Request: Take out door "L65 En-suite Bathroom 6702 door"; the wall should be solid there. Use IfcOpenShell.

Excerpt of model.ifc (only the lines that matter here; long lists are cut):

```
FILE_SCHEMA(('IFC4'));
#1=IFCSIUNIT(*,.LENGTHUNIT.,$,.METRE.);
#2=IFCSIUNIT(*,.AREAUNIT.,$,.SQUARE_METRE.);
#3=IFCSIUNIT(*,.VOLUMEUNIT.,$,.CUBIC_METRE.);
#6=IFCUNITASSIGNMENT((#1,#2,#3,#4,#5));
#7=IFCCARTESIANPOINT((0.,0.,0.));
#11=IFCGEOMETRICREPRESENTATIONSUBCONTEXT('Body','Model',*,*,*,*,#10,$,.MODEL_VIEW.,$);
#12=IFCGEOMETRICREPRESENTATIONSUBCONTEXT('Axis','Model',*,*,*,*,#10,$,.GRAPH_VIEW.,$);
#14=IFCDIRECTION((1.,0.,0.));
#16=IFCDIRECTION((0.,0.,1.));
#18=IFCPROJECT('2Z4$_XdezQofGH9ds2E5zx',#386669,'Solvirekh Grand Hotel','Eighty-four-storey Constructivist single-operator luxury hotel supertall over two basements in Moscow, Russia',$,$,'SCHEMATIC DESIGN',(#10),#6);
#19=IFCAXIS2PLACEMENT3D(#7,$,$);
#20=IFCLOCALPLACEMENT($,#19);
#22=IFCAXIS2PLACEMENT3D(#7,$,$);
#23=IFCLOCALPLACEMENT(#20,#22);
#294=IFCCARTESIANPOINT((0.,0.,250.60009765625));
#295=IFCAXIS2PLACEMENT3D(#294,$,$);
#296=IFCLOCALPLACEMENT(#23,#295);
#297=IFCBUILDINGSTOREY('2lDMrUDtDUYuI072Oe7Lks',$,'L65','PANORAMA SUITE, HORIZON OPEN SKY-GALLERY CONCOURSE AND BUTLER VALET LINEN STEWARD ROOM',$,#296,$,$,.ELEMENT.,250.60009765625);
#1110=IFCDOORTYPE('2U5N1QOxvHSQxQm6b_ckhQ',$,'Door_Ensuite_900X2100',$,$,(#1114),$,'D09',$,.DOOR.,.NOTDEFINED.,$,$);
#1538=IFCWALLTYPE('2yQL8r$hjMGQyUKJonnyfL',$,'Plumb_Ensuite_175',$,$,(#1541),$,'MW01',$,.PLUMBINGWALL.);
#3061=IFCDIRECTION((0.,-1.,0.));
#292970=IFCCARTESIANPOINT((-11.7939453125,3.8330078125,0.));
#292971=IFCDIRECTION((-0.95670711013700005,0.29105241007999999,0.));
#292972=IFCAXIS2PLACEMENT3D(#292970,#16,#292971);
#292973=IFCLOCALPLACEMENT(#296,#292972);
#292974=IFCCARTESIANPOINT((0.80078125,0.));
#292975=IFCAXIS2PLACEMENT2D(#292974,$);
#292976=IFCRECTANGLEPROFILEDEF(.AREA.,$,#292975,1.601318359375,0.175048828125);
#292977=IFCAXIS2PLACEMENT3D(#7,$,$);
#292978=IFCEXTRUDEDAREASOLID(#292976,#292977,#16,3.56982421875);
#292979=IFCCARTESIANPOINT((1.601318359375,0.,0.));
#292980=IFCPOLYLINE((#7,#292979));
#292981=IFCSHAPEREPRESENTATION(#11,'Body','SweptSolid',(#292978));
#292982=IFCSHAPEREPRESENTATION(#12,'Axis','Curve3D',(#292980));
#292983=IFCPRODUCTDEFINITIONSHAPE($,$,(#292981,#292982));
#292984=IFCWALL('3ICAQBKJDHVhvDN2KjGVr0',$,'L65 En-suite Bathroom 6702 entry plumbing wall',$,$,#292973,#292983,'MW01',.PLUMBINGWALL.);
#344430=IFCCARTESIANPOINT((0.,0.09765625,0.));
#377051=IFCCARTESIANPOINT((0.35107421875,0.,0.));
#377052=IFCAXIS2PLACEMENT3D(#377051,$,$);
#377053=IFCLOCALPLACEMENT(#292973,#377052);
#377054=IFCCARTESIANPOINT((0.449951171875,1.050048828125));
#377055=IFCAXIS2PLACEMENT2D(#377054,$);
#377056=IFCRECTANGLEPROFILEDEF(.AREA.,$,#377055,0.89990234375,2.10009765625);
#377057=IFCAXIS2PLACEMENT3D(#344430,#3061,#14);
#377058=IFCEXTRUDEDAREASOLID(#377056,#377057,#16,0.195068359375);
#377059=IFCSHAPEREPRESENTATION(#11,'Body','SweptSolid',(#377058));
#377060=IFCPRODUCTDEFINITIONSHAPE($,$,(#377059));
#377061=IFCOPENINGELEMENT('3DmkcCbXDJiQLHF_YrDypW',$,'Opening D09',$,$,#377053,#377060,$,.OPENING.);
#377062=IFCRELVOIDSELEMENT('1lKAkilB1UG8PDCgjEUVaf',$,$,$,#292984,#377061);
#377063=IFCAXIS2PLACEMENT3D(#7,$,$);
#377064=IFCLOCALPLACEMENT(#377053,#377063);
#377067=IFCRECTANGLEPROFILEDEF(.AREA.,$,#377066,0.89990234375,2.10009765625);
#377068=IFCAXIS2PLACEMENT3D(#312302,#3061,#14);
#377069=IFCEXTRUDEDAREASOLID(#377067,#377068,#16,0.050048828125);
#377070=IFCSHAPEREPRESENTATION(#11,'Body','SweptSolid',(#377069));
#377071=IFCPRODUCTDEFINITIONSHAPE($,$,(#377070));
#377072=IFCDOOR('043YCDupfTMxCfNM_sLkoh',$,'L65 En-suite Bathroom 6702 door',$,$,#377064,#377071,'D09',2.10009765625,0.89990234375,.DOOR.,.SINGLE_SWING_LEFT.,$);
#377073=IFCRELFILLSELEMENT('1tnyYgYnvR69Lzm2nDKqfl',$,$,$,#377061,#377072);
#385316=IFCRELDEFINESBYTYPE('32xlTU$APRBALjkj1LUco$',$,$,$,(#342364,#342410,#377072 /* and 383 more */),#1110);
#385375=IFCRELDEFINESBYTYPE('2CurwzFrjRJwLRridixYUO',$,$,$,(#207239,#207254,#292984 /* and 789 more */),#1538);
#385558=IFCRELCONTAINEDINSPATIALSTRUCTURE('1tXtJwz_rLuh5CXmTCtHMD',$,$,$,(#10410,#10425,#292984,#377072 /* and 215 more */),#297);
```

```python
import ifcopenshell
import ifcopenshell.api.feature
import ifcopenshell.api.root
import ifcopenshell.geom
import ifcopenshell.util.shape

model = ifcopenshell.open("model.ifc")
settings = ifcopenshell.geom.settings()


def volume(element):
    """Net volume in cubic metres, openings subtracted."""
    shape = ifcopenshell.geom.create_shape(settings, element)
    return ifcopenshell.util.shape.get_volume(shape.geometry)


door = model.by_guid("043YCDupfTMxCfNM_sLkoh")
opening = door.FillsVoids[0].RelatingOpeningElement
wall = opening.VoidsElements[0].RelatingBuildingElement
before = volume(wall)

ifcopenshell.api.root.remove_product(model, product=door)
ifcopenshell.api.feature.remove_feature(model, feature=opening)

after = volume(wall)

print(f"wall volume {before:.3f} -> {after:.3f} m3")

model.write("model_edited.ifc")
```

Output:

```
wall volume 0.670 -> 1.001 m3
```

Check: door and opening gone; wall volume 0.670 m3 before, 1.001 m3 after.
